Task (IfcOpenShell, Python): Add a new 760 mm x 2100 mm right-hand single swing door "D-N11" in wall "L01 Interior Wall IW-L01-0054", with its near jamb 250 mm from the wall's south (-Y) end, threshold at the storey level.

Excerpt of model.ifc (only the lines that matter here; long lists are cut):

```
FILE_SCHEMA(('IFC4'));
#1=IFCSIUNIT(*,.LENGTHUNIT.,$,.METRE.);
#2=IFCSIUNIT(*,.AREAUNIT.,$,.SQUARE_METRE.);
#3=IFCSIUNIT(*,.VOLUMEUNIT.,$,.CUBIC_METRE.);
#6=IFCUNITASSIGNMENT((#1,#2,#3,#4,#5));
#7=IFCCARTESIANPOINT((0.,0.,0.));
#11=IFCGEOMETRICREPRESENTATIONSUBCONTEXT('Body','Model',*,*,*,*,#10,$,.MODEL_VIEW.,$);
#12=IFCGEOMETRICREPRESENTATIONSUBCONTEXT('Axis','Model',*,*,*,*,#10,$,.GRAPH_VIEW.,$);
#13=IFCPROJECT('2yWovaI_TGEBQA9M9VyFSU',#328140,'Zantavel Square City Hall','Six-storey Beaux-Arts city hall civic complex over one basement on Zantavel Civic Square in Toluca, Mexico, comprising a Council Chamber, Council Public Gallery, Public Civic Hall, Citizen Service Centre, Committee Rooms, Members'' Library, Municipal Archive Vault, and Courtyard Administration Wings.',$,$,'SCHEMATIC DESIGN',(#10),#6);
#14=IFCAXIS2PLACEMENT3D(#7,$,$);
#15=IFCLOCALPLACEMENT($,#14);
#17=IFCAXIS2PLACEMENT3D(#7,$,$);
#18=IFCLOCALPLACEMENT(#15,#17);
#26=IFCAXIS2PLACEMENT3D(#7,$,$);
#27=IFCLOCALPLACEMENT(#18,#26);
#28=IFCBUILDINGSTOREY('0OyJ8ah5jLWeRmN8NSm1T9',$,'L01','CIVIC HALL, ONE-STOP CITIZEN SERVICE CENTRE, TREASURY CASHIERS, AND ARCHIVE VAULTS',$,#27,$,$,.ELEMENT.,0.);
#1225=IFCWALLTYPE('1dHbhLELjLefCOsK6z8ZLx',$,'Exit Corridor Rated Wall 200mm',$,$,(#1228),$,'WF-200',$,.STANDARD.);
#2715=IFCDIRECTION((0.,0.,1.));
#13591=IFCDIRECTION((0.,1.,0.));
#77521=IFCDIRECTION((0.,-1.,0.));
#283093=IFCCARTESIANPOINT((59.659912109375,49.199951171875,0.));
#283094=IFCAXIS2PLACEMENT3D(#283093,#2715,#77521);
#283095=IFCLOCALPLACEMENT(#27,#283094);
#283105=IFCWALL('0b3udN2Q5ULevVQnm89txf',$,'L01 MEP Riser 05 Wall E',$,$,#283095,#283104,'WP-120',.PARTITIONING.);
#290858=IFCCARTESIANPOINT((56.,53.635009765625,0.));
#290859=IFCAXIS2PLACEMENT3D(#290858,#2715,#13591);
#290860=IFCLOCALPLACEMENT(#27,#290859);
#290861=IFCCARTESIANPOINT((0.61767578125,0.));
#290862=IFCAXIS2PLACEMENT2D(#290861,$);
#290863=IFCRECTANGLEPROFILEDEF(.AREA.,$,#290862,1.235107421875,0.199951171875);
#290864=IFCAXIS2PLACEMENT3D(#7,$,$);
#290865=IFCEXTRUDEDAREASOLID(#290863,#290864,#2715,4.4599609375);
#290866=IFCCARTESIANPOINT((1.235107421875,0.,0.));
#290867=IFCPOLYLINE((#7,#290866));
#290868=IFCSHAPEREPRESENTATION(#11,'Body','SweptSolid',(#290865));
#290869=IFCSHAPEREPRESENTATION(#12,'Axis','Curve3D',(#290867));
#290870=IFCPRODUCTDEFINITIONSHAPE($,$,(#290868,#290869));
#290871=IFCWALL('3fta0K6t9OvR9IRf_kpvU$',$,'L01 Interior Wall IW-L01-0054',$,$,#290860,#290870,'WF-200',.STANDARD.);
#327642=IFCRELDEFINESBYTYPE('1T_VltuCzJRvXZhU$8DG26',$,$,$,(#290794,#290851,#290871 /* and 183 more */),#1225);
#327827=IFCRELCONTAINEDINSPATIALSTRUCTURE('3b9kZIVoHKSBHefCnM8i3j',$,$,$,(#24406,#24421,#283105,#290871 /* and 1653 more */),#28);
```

```python
import numpy as np
import ifcopenshell
import ifcopenshell.api.feature
import ifcopenshell.api.geometry
import ifcopenshell.api.root
import ifcopenshell.api.spatial
import ifcopenshell.geom
import ifcopenshell.util.element
import ifcopenshell.util.placement
import ifcopenshell.util.representation
import ifcopenshell.util.shape
import ifcopenshell.util.unit

model = ifcopenshell.open("model.ifc")
unit_scale = ifcopenshell.util.unit.calculate_unit_scale(model)
settings = ifcopenshell.geom.settings()


def volume(element):
    """Net volume in cubic metres, openings subtracted."""
    shape = ifcopenshell.geom.create_shape(settings, element)
    return ifcopenshell.util.shape.get_volume(shape.geometry)


wall = model.by_guid("3fta0K6t9OvR9IRf_kpvU$")
storey = ifcopenshell.util.element.get_container(wall, ifc_class="IfcBuildingStorey")
context = ifcopenshell.util.representation.get_context(model, "Model", "Body", "MODEL_VIEW")
before = volume(wall)

width, height, from_end, sill = 0.76, 2.1, 0.25, 0.0  # metres

# The wall runs along its own X axis, and the end named is its -X end.
wall_shape = ifcopenshell.geom.create_shape(settings, wall)
x, y, z = ifcopenshell.util.shape.get_vertices(wall_shape.geometry).T
start = x.min() + from_end
face, thickness = float(y.min()), float(y.max() - y.min())
wall_matrix = ifcopenshell.util.placement.get_local_placement(wall.ObjectPlacement)
level = ifcopenshell.util.placement.get_local_placement(storey.ObjectPlacement)[2, 3]


def in_wall(x, y):
    """Placement at x, y metres in the wall's axes, at sill height."""
    matrix = wall_matrix.copy()
    matrix[:, 3] = wall_matrix @ np.array([x / unit_scale, y / unit_scale, 0.0, 1.0])
    matrix[2, 3] = level + sill / unit_scale
    return matrix


# Opening: a box that overshoots both wall faces by 50 mm.
opening = ifcopenshell.api.root.create_entity(model, ifc_class="IfcOpeningElement", predefined_type="OPENING")
box = ifcopenshell.api.geometry.add_wall_representation(
    model, context=context, length=width, height=height, thickness=thickness + 0.1
)
ifcopenshell.api.geometry.assign_representation(model, product=opening, representation=box)
ifcopenshell.api.geometry.edit_object_placement(model, product=opening, matrix=in_wall(start, face - 0.05), is_si=False)
ifcopenshell.api.feature.add_feature(model, feature=opening, element=wall)

door = ifcopenshell.api.root.create_entity(model, ifc_class="IfcDoor", name="D-N11", predefined_type="DOOR")
door.OverallWidth, door.OverallHeight = width / unit_scale, height / unit_scale
door.OperationType = "SINGLE_SWING_RIGHT"
body = ifcopenshell.api.geometry.add_door_representation(
    model,
    context=context,
    overall_width=door.OverallWidth,
    overall_height=door.OverallHeight,
    operation_type="SINGLE_SWING_RIGHT",
    lining_properties={"LiningDepth": thickness / unit_scale, "ThresholdDepth": thickness / unit_scale},
)
ifcopenshell.api.geometry.assign_representation(model, product=door, representation=body)
ifcopenshell.api.spatial.assign_container(model, products=[door], relating_structure=storey)
ifcopenshell.api.feature.add_filling(model, opening=opening, element=door)

# The lining spans the wall, so the door starts at the wall face.
ifcopenshell.api.geometry.edit_object_placement(model, product=door, matrix=in_wall(start, face), is_si=False)

after = volume(wall)

print(f"wall volume {before:.3f} -> {after:.3f} m3")

model.write("model_v2.ifc")
```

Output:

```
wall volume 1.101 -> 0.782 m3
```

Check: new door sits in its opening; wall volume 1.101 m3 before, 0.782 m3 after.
